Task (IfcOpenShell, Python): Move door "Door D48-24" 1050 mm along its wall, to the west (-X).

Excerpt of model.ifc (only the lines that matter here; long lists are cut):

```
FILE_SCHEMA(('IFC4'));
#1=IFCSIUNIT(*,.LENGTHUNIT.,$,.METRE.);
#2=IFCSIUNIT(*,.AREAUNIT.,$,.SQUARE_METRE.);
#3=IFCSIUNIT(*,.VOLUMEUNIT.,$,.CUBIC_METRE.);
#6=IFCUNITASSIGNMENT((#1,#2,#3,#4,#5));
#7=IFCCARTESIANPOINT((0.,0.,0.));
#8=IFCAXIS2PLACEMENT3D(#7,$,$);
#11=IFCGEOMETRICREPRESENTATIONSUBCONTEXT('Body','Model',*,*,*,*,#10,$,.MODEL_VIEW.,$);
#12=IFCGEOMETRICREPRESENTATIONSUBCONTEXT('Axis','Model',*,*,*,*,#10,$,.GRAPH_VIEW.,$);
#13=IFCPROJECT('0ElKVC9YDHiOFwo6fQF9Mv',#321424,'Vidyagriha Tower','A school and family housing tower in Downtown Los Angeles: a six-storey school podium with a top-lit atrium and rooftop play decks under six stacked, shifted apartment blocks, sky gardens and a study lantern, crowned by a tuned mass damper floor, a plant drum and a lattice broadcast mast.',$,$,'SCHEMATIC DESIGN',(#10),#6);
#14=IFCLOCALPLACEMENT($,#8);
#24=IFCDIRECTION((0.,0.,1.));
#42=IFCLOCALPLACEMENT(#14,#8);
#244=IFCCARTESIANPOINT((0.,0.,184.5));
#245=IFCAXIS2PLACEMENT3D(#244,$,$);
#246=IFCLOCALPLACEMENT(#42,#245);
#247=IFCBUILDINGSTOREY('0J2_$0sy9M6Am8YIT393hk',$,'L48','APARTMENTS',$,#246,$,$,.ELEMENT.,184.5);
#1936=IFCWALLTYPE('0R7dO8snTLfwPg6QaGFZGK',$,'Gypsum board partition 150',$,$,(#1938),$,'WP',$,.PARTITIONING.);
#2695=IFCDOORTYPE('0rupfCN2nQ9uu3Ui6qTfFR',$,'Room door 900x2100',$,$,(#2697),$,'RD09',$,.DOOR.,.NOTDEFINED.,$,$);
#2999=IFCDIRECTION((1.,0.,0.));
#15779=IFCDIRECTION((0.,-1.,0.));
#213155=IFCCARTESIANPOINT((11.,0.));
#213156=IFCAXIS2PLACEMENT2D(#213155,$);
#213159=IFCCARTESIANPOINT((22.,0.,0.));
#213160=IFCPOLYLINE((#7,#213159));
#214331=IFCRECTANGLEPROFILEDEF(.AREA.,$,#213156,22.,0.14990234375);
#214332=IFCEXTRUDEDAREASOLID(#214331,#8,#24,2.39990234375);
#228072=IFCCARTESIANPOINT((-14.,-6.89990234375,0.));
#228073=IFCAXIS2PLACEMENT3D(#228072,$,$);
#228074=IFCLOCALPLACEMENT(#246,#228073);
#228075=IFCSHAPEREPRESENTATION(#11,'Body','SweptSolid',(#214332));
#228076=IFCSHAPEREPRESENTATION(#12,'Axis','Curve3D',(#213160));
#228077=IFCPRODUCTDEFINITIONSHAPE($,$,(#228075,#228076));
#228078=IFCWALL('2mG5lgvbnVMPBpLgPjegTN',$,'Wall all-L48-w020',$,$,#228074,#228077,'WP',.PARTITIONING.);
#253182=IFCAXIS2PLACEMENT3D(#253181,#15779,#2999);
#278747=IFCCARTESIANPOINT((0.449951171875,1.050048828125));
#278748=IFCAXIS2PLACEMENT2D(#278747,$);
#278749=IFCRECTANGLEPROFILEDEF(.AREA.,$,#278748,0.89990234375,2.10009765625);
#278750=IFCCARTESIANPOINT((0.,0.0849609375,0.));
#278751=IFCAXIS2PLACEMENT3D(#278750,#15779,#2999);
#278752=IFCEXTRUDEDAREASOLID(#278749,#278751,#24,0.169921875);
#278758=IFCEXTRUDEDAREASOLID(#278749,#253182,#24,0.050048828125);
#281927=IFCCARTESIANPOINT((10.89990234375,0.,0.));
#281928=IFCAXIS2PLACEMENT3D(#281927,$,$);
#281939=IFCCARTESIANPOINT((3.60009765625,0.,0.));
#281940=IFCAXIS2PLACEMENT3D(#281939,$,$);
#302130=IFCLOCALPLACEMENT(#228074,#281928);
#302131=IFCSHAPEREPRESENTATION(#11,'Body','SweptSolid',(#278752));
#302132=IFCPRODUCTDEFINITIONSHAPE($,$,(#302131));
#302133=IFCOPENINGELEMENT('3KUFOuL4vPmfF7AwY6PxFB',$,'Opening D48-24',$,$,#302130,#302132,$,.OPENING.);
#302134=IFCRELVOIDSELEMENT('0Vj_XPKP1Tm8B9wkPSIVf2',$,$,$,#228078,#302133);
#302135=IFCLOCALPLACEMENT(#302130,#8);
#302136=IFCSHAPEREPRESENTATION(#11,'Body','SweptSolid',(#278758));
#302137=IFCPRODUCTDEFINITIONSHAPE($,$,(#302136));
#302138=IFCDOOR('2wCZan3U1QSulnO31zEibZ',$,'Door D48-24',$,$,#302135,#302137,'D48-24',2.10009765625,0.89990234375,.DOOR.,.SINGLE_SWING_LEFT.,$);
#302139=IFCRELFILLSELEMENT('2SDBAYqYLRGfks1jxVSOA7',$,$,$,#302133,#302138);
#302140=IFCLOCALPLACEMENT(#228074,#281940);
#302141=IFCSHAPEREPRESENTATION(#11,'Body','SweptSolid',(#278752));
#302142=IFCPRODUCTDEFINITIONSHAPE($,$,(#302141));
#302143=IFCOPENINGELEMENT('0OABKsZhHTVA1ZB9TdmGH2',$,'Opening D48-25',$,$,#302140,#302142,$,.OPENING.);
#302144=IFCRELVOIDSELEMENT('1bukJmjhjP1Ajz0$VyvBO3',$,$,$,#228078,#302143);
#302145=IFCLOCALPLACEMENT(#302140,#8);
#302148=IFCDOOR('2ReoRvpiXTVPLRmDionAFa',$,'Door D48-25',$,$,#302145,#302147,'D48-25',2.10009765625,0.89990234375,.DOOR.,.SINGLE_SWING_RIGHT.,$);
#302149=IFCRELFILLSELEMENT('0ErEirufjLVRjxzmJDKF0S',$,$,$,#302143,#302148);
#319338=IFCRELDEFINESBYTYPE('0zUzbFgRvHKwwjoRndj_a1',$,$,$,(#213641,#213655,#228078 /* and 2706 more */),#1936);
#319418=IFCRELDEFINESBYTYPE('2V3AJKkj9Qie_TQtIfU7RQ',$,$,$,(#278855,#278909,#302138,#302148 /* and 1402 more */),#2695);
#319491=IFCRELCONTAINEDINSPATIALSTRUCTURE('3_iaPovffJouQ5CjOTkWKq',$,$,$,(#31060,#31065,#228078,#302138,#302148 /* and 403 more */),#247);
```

```python
import ifcopenshell
import ifcopenshell.api.geometry
import ifcopenshell.util.placement
import ifcopenshell.util.unit

model = ifcopenshell.open("model.ifc")
unit_scale = ifcopenshell.util.unit.calculate_unit_scale(model)

door = model.by_guid("2wCZan3U1QSulnO31zEibZ")
opening = door.FillsVoids[0].RelatingOpeningElement
wall = opening.VoidsElements[0].RelatingBuildingElement

wall_matrix = ifcopenshell.util.placement.get_local_placement(wall.ObjectPlacement)
shift = wall_matrix[:3, 0] * -1.05 / unit_scale
before = ifcopenshell.util.placement.get_local_placement(door.ObjectPlacement)[:3, 3].copy()

# The door is placed relative to its opening, so it follows when the opening moves.
matrix = ifcopenshell.util.placement.get_local_placement(opening.ObjectPlacement)
matrix[:3, 3] += shift
ifcopenshell.api.geometry.edit_object_placement(
    model, product=opening, matrix=matrix, is_si=False, should_transform_children=True
)

after = ifcopenshell.util.placement.get_local_placement(door.ObjectPlacement)[:3, 3]
print("door moved by", (after - before).round(3) + 0.0)

model.write("model_updated.ifc")
```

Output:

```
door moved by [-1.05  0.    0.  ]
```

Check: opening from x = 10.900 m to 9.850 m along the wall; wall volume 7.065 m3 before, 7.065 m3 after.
